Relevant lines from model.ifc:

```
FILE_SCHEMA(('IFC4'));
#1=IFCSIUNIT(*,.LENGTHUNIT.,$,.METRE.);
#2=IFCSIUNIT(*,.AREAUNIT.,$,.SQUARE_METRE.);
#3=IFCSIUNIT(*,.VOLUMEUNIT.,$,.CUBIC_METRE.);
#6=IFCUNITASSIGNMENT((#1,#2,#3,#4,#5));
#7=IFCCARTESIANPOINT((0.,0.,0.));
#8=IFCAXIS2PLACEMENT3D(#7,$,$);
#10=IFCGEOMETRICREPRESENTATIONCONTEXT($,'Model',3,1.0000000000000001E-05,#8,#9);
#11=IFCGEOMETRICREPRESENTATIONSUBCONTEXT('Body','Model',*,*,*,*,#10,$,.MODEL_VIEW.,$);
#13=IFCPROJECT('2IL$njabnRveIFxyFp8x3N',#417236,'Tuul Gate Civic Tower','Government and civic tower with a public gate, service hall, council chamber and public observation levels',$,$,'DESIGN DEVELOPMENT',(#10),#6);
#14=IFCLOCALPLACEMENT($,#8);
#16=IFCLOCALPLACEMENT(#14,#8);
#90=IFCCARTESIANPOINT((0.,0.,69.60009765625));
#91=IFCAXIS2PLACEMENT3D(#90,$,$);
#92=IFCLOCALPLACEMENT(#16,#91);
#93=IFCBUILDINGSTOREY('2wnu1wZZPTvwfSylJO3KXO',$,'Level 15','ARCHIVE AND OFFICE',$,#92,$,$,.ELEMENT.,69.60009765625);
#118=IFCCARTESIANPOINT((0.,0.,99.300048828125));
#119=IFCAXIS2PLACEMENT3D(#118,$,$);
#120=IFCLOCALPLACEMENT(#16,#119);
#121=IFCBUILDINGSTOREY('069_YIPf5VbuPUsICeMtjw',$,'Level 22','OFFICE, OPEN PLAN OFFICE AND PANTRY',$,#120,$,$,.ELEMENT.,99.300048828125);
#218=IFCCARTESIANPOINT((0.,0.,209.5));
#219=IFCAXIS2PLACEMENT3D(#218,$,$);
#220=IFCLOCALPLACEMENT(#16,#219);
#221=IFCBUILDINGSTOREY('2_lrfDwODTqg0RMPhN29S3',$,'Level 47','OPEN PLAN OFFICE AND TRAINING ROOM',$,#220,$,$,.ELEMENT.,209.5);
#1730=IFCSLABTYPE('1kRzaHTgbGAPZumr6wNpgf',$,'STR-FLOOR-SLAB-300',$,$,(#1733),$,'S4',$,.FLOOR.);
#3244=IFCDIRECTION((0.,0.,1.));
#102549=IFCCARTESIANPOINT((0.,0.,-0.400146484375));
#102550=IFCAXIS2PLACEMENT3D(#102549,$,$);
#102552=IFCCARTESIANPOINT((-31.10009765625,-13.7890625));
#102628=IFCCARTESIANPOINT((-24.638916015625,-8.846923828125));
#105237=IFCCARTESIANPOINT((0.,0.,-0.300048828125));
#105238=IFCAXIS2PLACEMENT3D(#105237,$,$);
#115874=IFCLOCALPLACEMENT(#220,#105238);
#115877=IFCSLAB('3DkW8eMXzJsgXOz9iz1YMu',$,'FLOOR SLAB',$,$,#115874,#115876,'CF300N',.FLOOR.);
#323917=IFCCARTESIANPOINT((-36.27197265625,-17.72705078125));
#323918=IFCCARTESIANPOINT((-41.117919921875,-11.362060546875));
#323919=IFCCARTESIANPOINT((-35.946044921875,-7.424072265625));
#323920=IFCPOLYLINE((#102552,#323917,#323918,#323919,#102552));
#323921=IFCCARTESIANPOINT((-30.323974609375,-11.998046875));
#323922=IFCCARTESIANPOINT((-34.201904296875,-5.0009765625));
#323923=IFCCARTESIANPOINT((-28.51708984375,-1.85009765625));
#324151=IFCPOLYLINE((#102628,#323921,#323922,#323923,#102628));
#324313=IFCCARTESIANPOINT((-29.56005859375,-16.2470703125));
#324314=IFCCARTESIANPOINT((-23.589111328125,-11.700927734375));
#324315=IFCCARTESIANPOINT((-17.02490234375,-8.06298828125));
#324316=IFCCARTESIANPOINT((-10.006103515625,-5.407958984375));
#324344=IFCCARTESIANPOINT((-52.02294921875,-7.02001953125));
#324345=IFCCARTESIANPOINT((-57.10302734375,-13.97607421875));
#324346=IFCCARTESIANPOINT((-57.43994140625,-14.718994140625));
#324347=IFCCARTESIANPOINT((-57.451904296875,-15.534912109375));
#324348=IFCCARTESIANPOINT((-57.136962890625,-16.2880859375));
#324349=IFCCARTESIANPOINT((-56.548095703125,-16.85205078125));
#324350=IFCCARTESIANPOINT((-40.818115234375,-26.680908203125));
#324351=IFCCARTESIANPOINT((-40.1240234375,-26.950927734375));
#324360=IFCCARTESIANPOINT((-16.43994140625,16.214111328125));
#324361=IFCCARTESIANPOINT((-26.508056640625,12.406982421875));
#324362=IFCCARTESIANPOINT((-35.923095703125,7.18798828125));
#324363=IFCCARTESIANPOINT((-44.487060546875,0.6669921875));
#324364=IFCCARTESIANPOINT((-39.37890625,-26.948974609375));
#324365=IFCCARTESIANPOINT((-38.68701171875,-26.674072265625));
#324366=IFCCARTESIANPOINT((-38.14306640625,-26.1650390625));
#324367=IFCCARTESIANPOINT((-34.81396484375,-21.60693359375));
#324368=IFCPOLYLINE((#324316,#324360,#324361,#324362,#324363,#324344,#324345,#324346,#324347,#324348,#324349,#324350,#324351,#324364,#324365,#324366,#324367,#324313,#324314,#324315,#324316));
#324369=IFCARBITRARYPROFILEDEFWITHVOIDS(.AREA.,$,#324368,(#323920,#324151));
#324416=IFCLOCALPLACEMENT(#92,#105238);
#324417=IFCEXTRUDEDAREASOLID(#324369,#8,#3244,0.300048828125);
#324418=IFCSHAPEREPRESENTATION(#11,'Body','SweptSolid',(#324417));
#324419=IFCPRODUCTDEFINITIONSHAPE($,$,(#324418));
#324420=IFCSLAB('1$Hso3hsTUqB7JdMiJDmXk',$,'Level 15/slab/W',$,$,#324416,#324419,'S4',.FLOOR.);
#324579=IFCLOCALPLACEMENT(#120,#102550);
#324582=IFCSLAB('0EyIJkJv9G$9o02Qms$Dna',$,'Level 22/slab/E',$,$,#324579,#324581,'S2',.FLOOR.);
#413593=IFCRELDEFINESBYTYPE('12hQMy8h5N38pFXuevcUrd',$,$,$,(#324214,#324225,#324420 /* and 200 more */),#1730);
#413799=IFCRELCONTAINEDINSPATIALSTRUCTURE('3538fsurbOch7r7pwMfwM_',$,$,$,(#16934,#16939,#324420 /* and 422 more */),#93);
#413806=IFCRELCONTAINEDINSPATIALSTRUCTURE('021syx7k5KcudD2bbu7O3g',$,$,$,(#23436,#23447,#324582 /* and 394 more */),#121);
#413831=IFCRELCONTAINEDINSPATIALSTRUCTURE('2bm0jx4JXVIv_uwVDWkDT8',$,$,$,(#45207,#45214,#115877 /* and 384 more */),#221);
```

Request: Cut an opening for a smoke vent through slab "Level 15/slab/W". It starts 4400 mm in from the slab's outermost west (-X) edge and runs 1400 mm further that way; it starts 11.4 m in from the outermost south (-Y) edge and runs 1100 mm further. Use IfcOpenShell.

```python
import numpy as np
import ifcopenshell
import ifcopenshell.api.feature
import ifcopenshell.api.geometry
import ifcopenshell.api.root
import ifcopenshell.geom
import ifcopenshell.util.placement
import ifcopenshell.util.representation
import ifcopenshell.util.shape
import ifcopenshell.util.unit

model = ifcopenshell.open("model.ifc")
unit_scale = ifcopenshell.util.unit.calculate_unit_scale(model)
settings = ifcopenshell.geom.settings()


def volume(element):
    """Net volume in cubic metres, openings subtracted."""
    shape = ifcopenshell.geom.create_shape(settings, element)
    return ifcopenshell.util.shape.get_volume(shape.geometry)


slab = model.by_guid("1$Hso3hsTUqB7JdMiJDmXk")
before = volume(slab)

# Extent in the slab's own axes, in metres. The edges named are its -X and -Y sides.
slab_shape = ifcopenshell.geom.create_shape(settings, slab)
vertices = ifcopenshell.util.shape.get_vertices(slab_shape.geometry)
x_min, y_min, bottom = vertices.min(axis=0)
top = vertices[:, 2].max()

opening = ifcopenshell.api.root.create_entity(model, ifc_class="IfcOpeningElement", name="Smoke vent opening", predefined_type="OPENING")
context = ifcopenshell.util.representation.get_context(model, "Model", "Body", "MODEL_VIEW")
width, depth = 1.4, 1.1
outline = [(0.0, 0.0), (width, 0.0), (width, depth), (0.0, depth), (0.0, 0.0)]
# Overshoot both faces by 50 mm so the cut is clean.
shape = ifcopenshell.api.geometry.add_slab_representation(
    model, context=context, depth=top - bottom + 0.1, polyline=outline
)
ifcopenshell.api.geometry.assign_representation(model, product=opening, representation=shape)

matrix = ifcopenshell.util.placement.get_local_placement(slab.ObjectPlacement)
matrix[:, 3] = matrix @ np.append(np.array([x_min + 4.4, y_min + 11.4, bottom - 0.05]) / unit_scale, 1.0)
ifcopenshell.api.geometry.edit_object_placement(model, product=opening, matrix=matrix, is_si=False)
ifcopenshell.api.feature.add_feature(model, feature=opening, element=slab)

after = volume(slab)

print(f"slab volume {before:.3f} -> {after:.3f} m3")

model.write("model_v2.ifc")
```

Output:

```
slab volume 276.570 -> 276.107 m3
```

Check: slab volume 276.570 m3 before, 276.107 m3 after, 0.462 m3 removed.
